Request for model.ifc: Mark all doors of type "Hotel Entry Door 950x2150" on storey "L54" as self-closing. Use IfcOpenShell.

First a look at what the model holds.

```python
import ifcopenshell
import ifcopenshell.util.element

model = ifcopenshell.open("model.ifc")
print(model.schema)
storey = next(s for s in model.by_type("IfcBuildingStorey") if s.Name == "L54")
doors = [e for e in ifcopenshell.util.element.get_decomposition(storey) if e.is_a("IfcDoor")]
seen = {}
for e in doors:
    element_type = ifcopenshell.util.element.get_type(e)
    key = (element_type.Name if element_type != e and element_type else None, ifcopenshell.util.element.get_pset(e, "Pset_DoorCommon", "SelfClosing"))
    seen[key] = seen.get(key, 0) + 1
for (name, value), count in sorted(seen.items(), key=str):
    print(count, "x", name, "|", value)
```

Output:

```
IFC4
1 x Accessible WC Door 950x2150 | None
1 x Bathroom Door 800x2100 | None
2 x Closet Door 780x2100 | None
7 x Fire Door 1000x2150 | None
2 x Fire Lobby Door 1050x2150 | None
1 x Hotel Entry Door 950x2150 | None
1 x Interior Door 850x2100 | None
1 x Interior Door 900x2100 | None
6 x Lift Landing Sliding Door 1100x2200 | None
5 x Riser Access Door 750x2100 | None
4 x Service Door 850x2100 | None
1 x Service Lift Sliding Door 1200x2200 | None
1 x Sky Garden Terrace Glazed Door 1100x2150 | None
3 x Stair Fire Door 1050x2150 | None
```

```python
import ifcopenshell
import ifcopenshell.api.pset
import ifcopenshell.util.element

model = ifcopenshell.open("model.ifc")

storey = next(s for s in model.by_type("IfcBuildingStorey") if s.Name == "L54")
doors = [e for e in ifcopenshell.util.element.get_decomposition(storey) if e.is_a("IfcDoor")]

count = 0
for e in doors:
    element_type = ifcopenshell.util.element.get_type(e)
    if element_type in (None, e) or element_type.Name != "Hotel Entry Door 950x2150":
        continue
    found = ifcopenshell.util.element.get_pset(e, "Pset_DoorCommon", should_inherit=False)
    if found:
        pset = model.by_id(found["id"])
        if len(ifcopenshell.util.element.get_elements_by_pset(pset)) > 1:
            pset = ifcopenshell.api.pset.unshare_pset(model, products=[e], pset=pset)[0]
    else:
        pset = ifcopenshell.api.pset.add_pset(model, product=e, name="Pset_DoorCommon")
    ifcopenshell.api.pset.edit_pset(model, pset=pset, properties={"SelfClosing": True})
    count += 1

print(count, "doors updated")

model.write("model_rev.ifc")
```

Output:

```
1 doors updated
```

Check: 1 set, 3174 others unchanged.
